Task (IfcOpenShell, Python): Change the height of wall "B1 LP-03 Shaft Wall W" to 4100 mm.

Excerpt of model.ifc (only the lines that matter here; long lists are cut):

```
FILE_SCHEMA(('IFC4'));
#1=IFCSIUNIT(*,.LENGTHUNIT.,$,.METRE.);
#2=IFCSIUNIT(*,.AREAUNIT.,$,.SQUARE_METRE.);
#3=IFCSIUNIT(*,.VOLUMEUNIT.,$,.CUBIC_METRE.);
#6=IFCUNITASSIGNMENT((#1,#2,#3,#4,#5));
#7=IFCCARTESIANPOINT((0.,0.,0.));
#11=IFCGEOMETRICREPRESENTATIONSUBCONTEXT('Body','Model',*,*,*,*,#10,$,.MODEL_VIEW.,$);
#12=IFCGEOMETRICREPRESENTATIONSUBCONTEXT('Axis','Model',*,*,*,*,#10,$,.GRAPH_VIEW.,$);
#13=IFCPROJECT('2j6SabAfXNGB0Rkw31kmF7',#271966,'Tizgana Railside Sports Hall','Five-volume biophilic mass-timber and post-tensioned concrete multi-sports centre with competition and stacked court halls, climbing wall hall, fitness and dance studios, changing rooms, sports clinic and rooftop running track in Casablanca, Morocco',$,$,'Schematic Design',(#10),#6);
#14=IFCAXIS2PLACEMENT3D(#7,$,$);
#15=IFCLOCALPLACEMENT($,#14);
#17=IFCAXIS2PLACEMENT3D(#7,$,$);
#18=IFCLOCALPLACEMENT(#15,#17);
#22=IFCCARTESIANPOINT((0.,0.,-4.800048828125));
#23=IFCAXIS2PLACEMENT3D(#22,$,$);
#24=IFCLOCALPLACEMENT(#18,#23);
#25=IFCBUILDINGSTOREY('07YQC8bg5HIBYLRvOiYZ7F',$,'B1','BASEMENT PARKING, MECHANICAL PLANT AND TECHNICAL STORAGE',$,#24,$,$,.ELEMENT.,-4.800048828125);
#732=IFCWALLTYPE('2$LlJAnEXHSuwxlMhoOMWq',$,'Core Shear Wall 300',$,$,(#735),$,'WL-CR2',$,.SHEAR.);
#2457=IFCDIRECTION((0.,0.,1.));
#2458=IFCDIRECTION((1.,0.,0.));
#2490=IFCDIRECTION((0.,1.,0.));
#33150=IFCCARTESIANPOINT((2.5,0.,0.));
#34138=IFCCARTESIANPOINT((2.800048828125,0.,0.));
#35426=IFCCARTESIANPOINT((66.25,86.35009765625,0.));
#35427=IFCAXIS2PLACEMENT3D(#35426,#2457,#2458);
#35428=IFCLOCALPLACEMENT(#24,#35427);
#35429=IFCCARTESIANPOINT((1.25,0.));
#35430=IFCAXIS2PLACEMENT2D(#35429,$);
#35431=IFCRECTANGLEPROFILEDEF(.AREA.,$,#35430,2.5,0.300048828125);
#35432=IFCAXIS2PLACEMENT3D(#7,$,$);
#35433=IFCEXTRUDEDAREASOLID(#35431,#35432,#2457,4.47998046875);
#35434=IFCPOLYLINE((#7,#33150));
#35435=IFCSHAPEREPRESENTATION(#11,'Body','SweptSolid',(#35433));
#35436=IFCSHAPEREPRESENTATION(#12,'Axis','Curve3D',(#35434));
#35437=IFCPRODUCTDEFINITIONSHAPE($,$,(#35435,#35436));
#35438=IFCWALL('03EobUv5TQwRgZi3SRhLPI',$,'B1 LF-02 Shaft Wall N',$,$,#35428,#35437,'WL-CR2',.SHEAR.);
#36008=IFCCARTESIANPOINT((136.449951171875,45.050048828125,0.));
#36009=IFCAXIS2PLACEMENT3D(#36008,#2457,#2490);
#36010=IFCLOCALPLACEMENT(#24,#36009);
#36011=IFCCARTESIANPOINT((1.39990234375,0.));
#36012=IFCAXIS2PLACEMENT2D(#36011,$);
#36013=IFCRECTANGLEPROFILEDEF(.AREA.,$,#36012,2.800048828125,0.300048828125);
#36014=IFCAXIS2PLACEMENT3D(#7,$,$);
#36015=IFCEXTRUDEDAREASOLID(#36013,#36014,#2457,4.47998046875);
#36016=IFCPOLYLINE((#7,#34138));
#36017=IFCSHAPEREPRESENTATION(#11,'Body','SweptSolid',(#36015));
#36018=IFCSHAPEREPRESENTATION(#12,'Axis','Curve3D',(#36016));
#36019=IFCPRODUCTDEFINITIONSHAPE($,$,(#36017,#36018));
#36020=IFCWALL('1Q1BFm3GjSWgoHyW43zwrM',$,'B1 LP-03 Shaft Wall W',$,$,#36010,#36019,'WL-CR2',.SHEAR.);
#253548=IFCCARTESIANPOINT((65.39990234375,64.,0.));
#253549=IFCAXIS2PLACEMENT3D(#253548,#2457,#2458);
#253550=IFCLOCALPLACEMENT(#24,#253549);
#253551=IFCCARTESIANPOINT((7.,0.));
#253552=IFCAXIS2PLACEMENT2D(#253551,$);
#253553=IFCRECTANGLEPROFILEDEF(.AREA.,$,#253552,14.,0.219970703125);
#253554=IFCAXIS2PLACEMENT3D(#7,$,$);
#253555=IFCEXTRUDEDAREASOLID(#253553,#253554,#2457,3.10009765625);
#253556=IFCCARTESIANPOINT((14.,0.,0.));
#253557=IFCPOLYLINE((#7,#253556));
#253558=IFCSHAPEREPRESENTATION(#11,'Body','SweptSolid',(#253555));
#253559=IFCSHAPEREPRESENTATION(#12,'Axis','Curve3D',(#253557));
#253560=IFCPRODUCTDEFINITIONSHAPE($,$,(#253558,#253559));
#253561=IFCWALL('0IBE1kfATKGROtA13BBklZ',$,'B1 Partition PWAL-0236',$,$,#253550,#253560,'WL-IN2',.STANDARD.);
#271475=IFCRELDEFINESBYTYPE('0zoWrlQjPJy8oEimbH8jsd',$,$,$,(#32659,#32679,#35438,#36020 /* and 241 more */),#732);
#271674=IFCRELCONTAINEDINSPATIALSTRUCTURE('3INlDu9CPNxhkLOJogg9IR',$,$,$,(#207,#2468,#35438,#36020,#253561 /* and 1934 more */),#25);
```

```python
import ifcopenshell
import ifcopenshell.geom
import ifcopenshell.util.representation
import ifcopenshell.util.shape

model = ifcopenshell.open("model.ifc")
settings = ifcopenshell.geom.settings()


def volume(element):
    """Net volume in cubic metres, openings subtracted."""
    shape = ifcopenshell.geom.create_shape(settings, element)
    return ifcopenshell.util.shape.get_volume(shape.geometry)


wall = model.by_id(36020)
before = volume(wall)

body = ifcopenshell.util.representation.get_representation(wall, "Model", "Body")
solid = body.Items[0]
old_height = solid.Depth
solid.Depth = 4.1
after = volume(wall)

print(f"height {old_height:g} -> {solid.Depth:g}, volume {before:.3f} -> {after:.3f} m3")

model.write("model_v2.ifc")
```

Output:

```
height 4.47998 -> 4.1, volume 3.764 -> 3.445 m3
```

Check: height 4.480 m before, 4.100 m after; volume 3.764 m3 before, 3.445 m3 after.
